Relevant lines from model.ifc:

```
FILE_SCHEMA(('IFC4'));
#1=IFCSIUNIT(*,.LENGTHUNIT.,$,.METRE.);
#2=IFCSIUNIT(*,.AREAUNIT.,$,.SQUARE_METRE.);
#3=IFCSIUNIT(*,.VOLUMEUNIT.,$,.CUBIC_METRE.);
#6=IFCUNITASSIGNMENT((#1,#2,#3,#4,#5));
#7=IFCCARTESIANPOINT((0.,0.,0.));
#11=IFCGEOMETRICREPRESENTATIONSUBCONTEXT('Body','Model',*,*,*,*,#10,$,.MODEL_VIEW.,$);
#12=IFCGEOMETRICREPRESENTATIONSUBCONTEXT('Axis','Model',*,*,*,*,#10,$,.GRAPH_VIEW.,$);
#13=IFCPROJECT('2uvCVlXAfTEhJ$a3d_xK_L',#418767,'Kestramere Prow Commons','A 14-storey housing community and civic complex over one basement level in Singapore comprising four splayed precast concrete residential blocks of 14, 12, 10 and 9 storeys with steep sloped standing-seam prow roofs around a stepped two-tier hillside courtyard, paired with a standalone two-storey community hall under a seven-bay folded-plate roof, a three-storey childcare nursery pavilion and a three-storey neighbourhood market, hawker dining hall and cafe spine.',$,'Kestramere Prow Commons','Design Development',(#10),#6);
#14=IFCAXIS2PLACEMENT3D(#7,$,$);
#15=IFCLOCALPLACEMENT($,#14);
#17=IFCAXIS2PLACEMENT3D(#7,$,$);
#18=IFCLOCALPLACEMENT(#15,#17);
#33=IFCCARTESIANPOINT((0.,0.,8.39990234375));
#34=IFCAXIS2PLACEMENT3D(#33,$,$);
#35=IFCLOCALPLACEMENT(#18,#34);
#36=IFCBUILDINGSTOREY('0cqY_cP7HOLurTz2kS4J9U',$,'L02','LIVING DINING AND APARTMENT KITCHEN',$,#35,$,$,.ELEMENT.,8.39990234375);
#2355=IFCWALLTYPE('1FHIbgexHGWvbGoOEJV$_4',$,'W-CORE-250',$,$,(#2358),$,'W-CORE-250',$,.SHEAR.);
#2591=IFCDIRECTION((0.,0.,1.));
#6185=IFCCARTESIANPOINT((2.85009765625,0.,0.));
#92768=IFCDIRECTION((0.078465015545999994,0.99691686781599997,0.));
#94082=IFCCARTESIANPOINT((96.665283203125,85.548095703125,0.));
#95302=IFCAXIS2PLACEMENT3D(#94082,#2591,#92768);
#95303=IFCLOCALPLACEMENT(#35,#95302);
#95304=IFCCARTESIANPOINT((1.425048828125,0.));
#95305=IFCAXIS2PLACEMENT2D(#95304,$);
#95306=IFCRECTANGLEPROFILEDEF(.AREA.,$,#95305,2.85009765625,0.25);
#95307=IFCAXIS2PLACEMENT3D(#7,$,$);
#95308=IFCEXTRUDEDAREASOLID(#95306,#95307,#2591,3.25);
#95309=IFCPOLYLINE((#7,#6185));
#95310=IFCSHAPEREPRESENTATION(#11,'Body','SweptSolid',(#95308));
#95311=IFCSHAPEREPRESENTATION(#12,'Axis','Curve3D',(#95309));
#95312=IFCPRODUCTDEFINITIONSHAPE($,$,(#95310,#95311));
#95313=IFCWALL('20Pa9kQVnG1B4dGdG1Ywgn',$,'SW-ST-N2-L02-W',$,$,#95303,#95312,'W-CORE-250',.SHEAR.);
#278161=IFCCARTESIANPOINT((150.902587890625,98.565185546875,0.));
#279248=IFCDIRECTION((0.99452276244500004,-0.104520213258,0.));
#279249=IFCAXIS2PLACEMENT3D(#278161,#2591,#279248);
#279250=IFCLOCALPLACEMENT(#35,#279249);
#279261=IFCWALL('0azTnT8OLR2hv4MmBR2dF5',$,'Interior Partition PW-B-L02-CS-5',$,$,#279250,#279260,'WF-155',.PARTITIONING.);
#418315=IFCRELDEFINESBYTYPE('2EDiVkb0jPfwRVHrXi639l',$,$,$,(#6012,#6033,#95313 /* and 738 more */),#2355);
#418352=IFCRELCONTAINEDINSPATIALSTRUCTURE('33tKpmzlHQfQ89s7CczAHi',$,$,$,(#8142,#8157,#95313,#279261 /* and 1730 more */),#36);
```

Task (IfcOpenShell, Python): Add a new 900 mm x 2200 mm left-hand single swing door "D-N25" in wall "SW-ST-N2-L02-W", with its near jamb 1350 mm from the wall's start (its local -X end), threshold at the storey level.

```python
import numpy as np
import ifcopenshell
import ifcopenshell.api.feature
import ifcopenshell.api.geometry
import ifcopenshell.api.root
import ifcopenshell.api.spatial
import ifcopenshell.geom
import ifcopenshell.util.element
import ifcopenshell.util.placement
import ifcopenshell.util.representation
import ifcopenshell.util.shape
import ifcopenshell.util.unit

model = ifcopenshell.open("model.ifc")
unit_scale = ifcopenshell.util.unit.calculate_unit_scale(model)
settings = ifcopenshell.geom.settings()


def volume(element):
    """Net volume in cubic metres, openings subtracted."""
    shape = ifcopenshell.geom.create_shape(settings, element)
    return ifcopenshell.util.shape.get_volume(shape.geometry)


wall = model.by_guid("20Pa9kQVnG1B4dGdG1Ywgn")
storey = ifcopenshell.util.element.get_container(wall, ifc_class="IfcBuildingStorey")
context = ifcopenshell.util.representation.get_context(model, "Model", "Body", "MODEL_VIEW")
before = volume(wall)

width, height, from_end, sill = 0.9, 2.2, 1.35, 0.0  # metres

# The wall runs along its own X axis, and the end named is its -X end.
wall_shape = ifcopenshell.geom.create_shape(settings, wall)
x, y, z = ifcopenshell.util.shape.get_vertices(wall_shape.geometry).T
start = x.min() + from_end
face, thickness = float(y.min()), float(y.max() - y.min())
wall_matrix = ifcopenshell.util.placement.get_local_placement(wall.ObjectPlacement)
level = ifcopenshell.util.placement.get_local_placement(storey.ObjectPlacement)[2, 3]


def in_wall(x, y):
    """Placement at x, y metres in the wall's axes, at sill height."""
    matrix = wall_matrix.copy()
    matrix[:, 3] = wall_matrix @ np.array([x / unit_scale, y / unit_scale, 0.0, 1.0])
    matrix[2, 3] = level + sill / unit_scale
    return matrix


# Opening: a box that overshoots both wall faces by 50 mm.
opening = ifcopenshell.api.root.create_entity(model, ifc_class="IfcOpeningElement", predefined_type="OPENING")
box = ifcopenshell.api.geometry.add_wall_representation(
    model, context=context, length=width, height=height, thickness=thickness + 0.1
)
ifcopenshell.api.geometry.assign_representation(model, product=opening, representation=box)
ifcopenshell.api.geometry.edit_object_placement(model, product=opening, matrix=in_wall(start, face - 0.05), is_si=False)
ifcopenshell.api.feature.add_feature(model, feature=opening, element=wall)

door = ifcopenshell.api.root.create_entity(model, ifc_class="IfcDoor", name="D-N25", predefined_type="DOOR")
door.OverallWidth, door.OverallHeight = width / unit_scale, height / unit_scale
door.OperationType = "SINGLE_SWING_LEFT"
body = ifcopenshell.api.geometry.add_door_representation(
    model,
    context=context,
    overall_width=door.OverallWidth,
    overall_height=door.OverallHeight,
    operation_type="SINGLE_SWING_LEFT",
    lining_properties={"LiningDepth": thickness / unit_scale, "ThresholdDepth": thickness / unit_scale},
)
ifcopenshell.api.geometry.assign_representation(model, product=door, representation=body)
ifcopenshell.api.spatial.assign_container(model, products=[door], relating_structure=storey)
ifcopenshell.api.feature.add_filling(model, opening=opening, element=door)

# The lining spans the wall, so the door starts at the wall face.
ifcopenshell.api.geometry.edit_object_placement(model, product=door, matrix=in_wall(start, face), is_si=False)

after = volume(wall)

print(f"wall volume {before:.3f} -> {after:.3f} m3")

model.write("model_v2.ifc")
```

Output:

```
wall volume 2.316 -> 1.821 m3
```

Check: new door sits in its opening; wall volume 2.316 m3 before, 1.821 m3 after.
